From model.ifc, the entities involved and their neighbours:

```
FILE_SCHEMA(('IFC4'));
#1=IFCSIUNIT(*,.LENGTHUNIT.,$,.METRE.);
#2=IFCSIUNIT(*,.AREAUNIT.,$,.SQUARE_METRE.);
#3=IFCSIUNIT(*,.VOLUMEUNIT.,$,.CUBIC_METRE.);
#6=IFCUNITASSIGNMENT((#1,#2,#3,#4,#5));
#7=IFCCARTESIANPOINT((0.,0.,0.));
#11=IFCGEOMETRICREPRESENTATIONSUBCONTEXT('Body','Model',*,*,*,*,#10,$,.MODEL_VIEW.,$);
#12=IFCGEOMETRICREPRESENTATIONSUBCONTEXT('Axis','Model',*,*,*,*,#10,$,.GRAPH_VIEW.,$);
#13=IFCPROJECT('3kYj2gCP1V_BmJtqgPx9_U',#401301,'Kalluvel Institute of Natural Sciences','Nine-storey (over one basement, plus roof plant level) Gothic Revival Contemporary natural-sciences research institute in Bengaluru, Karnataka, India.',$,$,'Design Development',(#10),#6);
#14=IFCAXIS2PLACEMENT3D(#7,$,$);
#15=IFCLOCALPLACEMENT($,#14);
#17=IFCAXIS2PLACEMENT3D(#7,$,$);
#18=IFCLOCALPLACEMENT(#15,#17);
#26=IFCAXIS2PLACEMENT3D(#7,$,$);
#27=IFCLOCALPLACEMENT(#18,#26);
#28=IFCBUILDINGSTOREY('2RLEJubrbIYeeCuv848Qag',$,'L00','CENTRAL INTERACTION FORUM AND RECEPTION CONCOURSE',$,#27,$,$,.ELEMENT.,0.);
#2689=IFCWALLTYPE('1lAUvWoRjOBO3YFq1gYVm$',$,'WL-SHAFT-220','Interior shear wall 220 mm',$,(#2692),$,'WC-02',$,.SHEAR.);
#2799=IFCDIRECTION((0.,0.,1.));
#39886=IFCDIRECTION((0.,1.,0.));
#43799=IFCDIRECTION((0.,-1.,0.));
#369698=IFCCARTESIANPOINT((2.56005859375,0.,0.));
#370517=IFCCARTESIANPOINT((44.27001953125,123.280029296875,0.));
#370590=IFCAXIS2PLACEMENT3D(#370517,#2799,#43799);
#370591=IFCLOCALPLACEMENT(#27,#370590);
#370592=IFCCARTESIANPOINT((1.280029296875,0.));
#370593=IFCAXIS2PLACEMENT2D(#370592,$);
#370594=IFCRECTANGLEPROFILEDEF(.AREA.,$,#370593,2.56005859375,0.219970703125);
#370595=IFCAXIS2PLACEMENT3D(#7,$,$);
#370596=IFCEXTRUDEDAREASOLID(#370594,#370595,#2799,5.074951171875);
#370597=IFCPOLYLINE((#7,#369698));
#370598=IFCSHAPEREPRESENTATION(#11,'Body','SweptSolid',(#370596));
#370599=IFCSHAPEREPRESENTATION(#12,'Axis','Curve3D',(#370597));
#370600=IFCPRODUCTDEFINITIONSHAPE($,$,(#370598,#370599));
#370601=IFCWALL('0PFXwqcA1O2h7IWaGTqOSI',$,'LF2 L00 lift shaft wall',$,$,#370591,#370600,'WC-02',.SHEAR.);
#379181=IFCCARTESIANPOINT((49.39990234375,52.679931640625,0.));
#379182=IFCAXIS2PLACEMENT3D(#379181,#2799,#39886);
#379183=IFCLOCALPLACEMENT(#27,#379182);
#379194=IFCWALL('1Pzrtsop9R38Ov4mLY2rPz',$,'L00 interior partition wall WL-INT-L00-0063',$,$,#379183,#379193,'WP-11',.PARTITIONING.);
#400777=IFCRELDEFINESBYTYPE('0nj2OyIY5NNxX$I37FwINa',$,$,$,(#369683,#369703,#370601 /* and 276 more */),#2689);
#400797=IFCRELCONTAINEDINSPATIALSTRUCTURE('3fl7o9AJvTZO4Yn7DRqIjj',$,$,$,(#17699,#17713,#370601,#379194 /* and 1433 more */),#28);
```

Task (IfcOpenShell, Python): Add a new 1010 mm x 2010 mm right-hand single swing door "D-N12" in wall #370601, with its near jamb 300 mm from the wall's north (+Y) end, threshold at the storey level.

```python
import numpy as np
import ifcopenshell
import ifcopenshell.api.feature
import ifcopenshell.api.geometry
import ifcopenshell.api.root
import ifcopenshell.api.spatial
import ifcopenshell.geom
import ifcopenshell.util.element
import ifcopenshell.util.placement
import ifcopenshell.util.representation
import ifcopenshell.util.shape
import ifcopenshell.util.unit

model = ifcopenshell.open("model.ifc")
unit_scale = ifcopenshell.util.unit.calculate_unit_scale(model)
settings = ifcopenshell.geom.settings()


def volume(element):
    """Net volume in cubic metres, openings subtracted."""
    shape = ifcopenshell.geom.create_shape(settings, element)
    return ifcopenshell.util.shape.get_volume(shape.geometry)


wall = model.by_guid("0PFXwqcA1O2h7IWaGTqOSI")
storey = ifcopenshell.util.element.get_container(wall, ifc_class="IfcBuildingStorey")
context = ifcopenshell.util.representation.get_context(model, "Model", "Body", "MODEL_VIEW")
before = volume(wall)

width, height, from_end, sill = 1.01, 2.01, 0.3, 0.0  # metres

# The wall runs along its own X axis, and the end named is its -X end.
wall_shape = ifcopenshell.geom.create_shape(settings, wall)
x, y, z = ifcopenshell.util.shape.get_vertices(wall_shape.geometry).T
start = x.min() + from_end
face, thickness = float(y.min()), float(y.max() - y.min())
wall_matrix = ifcopenshell.util.placement.get_local_placement(wall.ObjectPlacement)
level = ifcopenshell.util.placement.get_local_placement(storey.ObjectPlacement)[2, 3]


def in_wall(x, y):
    """Placement at x, y metres in the wall's axes, at sill height."""
    matrix = wall_matrix.copy()
    matrix[:, 3] = wall_matrix @ np.array([x / unit_scale, y / unit_scale, 0.0, 1.0])
    matrix[2, 3] = level + sill / unit_scale
    return matrix


# Opening: a box that overshoots both wall faces by 50 mm.
opening = ifcopenshell.api.root.create_entity(model, ifc_class="IfcOpeningElement", predefined_type="OPENING")
box = ifcopenshell.api.geometry.add_wall_representation(
    model, context=context, length=width, height=height, thickness=thickness + 0.1
)
ifcopenshell.api.geometry.assign_representation(model, product=opening, representation=box)
ifcopenshell.api.geometry.edit_object_placement(model, product=opening, matrix=in_wall(start, face - 0.05), is_si=False)
ifcopenshell.api.feature.add_feature(model, feature=opening, element=wall)

door = ifcopenshell.api.root.create_entity(model, ifc_class="IfcDoor", name="D-N12", predefined_type="DOOR")
door.OverallWidth, door.OverallHeight = width / unit_scale, height / unit_scale
door.OperationType = "SINGLE_SWING_RIGHT"
body = ifcopenshell.api.geometry.add_door_representation(
    model,
    context=context,
    overall_width=door.OverallWidth,
    overall_height=door.OverallHeight,
    operation_type="SINGLE_SWING_RIGHT",
    lining_properties={"LiningDepth": thickness / unit_scale, "ThresholdDepth": thickness / unit_scale},
)
ifcopenshell.api.geometry.assign_representation(model, product=door, representation=body)
ifcopenshell.api.spatial.assign_container(model, products=[door], relating_structure=storey)
ifcopenshell.api.feature.add_filling(model, opening=opening, element=door)

# The lining spans the wall, so the door starts at the wall face.
ifcopenshell.api.geometry.edit_object_placement(model, product=door, matrix=in_wall(start, face), is_si=False)

after = volume(wall)

print(f"wall volume {before:.3f} -> {after:.3f} m3")

model.write("model_updated.ifc")
```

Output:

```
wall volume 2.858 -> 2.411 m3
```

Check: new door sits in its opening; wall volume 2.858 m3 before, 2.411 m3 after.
